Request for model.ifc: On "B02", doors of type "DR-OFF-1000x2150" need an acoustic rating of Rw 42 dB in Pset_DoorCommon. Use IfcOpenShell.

First a look at what the model holds.

```python
import ifcopenshell
import ifcopenshell.util.element

model = ifcopenshell.open("model.ifc")
print(model.schema)
storey = next(s for s in model.by_type("IfcBuildingStorey") if s.Name == "B02")
doors = [e for e in ifcopenshell.util.element.get_decomposition(storey) if e.is_a("IfcDoor")]
seen = {}
for e in doors:
    element_type = ifcopenshell.util.element.get_type(e)
    key = (element_type.Name if element_type != e and element_type else None, ifcopenshell.util.element.get_pset(e, "Pset_DoorCommon", "AcousticRating"))
    seen[key] = seen.get(key, 0) + 1
for (name, value), count in sorted(seen.items(), key=str):
    print(count, "x", name, "|", value)
```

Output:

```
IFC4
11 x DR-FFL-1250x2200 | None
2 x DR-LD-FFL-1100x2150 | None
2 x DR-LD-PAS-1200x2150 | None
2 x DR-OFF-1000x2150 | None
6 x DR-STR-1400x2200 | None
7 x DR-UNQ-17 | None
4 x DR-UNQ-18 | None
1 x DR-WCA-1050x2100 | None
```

```python
import ifcopenshell
import ifcopenshell.api.pset
import ifcopenshell.util.element

model = ifcopenshell.open("model.ifc")

storey = next(s for s in model.by_type("IfcBuildingStorey") if s.Name == "B02")
doors = [e for e in ifcopenshell.util.element.get_decomposition(storey) if e.is_a("IfcDoor")]

count = 0
for e in doors:
    element_type = ifcopenshell.util.element.get_type(e)
    if element_type in (None, e) or element_type.Name != "DR-OFF-1000x2150":
        continue
    # add_pset returns the element's existing set when there is one.
    pset = ifcopenshell.api.pset.add_pset(model, product=e, name="Pset_DoorCommon")
    ifcopenshell.api.pset.edit_pset(model, pset=pset, properties={"AcousticRating": "Rw 42 dB"})
    count += 1

print(count, "doors updated")

model.write("model_rev.ifc")
```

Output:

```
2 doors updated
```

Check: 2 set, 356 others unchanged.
